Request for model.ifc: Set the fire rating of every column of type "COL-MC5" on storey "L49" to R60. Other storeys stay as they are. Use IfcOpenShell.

First a look at what the model holds.

```python
import ifcopenshell
import ifcopenshell.util.element

model = ifcopenshell.open("model.ifc")
print(model.schema)
storey = next(s for s in model.by_type("IfcBuildingStorey") if s.Name == "L49")
columns = [e for e in ifcopenshell.util.element.get_decomposition(storey) if e.is_a("IfcColumn")]
seen = {}
for e in columns:
    element_type = ifcopenshell.util.element.get_type(e)
    key = (element_type.Name if element_type != e and element_type else None, ifcopenshell.util.element.get_pset(e, "Pset_ColumnCommon", "FireRating"))
    seen[key] = seen.get(key, 0) + 1
for (name, value), count in sorted(seen.items(), key=str):
    print(count, "x", name, "|", value)
```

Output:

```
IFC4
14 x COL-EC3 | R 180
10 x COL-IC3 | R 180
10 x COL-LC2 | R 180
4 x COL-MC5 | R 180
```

```python
import ifcopenshell
import ifcopenshell.api.pset
import ifcopenshell.util.element

model = ifcopenshell.open("model.ifc")

storey = next(s for s in model.by_type("IfcBuildingStorey") if s.Name == "L49")
columns = [e for e in ifcopenshell.util.element.get_decomposition(storey) if e.is_a("IfcColumn")]

count = 0
for e in columns:
    element_type = ifcopenshell.util.element.get_type(e)
    if element_type in (None, e) or element_type.Name != "COL-MC5":
        continue
    found = ifcopenshell.util.element.get_pset(e, "Pset_ColumnCommon", should_inherit=False)
    if found:
        pset = model.by_id(found["id"])
        if len(ifcopenshell.util.element.get_elements_by_pset(pset)) > 1:
            pset = ifcopenshell.api.pset.unshare_pset(model, products=[e], pset=pset)[0]
    else:
        pset = ifcopenshell.api.pset.add_pset(model, product=e, name="Pset_ColumnCommon")
    ifcopenshell.api.pset.edit_pset(model, pset=pset, properties={"FireRating": "R60"})
    count += 1

print(count, "columns updated")

model.write("model_rev.ifc")
```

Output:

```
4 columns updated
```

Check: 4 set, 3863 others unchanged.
